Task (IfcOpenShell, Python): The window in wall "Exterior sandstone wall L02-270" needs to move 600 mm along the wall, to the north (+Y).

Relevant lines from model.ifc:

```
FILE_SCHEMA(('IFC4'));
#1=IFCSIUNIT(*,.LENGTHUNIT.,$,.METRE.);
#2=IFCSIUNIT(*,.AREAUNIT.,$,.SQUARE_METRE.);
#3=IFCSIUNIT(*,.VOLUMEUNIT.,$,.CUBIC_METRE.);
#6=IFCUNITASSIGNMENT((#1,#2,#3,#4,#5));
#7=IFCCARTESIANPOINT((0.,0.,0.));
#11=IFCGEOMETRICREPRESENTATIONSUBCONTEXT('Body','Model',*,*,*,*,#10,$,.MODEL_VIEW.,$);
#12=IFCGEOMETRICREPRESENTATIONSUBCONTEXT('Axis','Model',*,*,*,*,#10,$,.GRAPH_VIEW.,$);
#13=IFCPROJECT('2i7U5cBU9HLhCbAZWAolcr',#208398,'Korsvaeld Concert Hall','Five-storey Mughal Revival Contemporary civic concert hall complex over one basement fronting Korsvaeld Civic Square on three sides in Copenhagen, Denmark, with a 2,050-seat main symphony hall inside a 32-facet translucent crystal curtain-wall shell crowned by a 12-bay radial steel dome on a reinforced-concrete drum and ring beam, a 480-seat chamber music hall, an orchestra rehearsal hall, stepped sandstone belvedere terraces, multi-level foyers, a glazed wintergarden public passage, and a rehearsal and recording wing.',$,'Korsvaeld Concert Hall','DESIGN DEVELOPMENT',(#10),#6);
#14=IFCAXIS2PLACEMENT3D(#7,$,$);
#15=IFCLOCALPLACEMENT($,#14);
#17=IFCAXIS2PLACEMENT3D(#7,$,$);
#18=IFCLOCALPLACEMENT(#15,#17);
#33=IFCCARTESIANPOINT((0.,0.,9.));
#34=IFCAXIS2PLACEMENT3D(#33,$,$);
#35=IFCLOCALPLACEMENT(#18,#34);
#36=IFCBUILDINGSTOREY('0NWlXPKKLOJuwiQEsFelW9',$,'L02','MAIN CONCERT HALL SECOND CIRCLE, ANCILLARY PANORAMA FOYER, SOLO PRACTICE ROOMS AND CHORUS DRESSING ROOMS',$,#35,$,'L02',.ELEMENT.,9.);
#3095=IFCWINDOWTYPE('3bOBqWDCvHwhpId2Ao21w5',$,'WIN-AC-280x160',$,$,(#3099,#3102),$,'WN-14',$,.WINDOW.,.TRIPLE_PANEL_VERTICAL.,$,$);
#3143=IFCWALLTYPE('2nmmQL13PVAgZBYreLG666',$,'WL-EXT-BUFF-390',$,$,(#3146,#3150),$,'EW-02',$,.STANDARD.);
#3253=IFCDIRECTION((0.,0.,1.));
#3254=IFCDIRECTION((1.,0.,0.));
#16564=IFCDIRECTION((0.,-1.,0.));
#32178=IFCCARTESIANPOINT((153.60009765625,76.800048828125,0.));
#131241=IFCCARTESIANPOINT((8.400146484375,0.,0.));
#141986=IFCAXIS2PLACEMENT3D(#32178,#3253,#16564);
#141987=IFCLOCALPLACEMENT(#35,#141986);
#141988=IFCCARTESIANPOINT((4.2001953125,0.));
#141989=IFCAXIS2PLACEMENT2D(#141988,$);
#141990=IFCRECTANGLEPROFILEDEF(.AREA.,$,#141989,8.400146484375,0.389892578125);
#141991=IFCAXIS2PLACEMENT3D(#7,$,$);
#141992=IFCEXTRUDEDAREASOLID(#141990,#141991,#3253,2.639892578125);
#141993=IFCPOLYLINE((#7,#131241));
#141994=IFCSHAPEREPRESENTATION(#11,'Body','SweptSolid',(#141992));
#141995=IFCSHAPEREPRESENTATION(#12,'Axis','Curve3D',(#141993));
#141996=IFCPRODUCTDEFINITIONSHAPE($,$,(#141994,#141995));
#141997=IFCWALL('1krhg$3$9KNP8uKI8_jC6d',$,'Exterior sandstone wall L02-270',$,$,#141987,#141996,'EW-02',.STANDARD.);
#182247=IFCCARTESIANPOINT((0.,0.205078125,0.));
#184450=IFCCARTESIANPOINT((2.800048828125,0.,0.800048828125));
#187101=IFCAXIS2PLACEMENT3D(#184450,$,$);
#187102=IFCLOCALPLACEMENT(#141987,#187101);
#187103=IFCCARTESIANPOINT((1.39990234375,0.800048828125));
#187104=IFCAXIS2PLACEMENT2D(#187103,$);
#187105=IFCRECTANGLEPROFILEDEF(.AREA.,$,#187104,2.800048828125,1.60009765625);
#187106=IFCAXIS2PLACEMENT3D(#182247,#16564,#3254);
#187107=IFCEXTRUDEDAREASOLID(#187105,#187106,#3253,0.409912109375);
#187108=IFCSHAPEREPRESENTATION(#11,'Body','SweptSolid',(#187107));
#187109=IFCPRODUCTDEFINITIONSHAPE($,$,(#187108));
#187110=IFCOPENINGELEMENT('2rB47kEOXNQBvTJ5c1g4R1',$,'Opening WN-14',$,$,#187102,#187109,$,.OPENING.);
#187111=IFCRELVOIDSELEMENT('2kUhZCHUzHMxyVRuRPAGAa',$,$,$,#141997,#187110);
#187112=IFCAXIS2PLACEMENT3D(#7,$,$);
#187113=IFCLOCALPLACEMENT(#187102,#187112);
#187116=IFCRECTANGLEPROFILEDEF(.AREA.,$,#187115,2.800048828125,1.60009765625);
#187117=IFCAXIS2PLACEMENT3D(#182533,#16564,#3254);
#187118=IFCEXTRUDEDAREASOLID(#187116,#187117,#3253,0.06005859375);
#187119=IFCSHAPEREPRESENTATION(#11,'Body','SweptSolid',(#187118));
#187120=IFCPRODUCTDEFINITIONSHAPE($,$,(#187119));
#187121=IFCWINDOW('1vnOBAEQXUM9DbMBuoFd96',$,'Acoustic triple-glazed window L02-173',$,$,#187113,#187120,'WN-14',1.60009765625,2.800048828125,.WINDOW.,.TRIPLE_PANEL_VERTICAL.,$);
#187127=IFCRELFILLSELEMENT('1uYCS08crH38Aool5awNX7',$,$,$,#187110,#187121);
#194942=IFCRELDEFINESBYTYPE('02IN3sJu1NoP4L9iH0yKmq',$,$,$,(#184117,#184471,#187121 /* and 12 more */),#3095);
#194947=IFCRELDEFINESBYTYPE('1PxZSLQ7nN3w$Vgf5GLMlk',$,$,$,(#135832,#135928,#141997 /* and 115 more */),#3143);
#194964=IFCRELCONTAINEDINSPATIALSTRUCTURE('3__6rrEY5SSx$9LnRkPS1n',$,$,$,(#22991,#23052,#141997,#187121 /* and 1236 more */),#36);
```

```python
import ifcopenshell
import ifcopenshell.api.geometry
import ifcopenshell.util.placement

model = ifcopenshell.open("model.ifc")

window = model.by_guid("1vnOBAEQXUM9DbMBuoFd96")
opening = window.FillsVoids[0].RelatingOpeningElement
wall = opening.VoidsElements[0].RelatingBuildingElement

wall_matrix = ifcopenshell.util.placement.get_local_placement(wall.ObjectPlacement)
shift = wall_matrix[:3, 0] * -0.6
before = ifcopenshell.util.placement.get_local_placement(window.ObjectPlacement)[:3, 3].copy()

# The window is placed relative to its opening, so it follows when the opening moves.
matrix = ifcopenshell.util.placement.get_local_placement(opening.ObjectPlacement)
matrix[:3, 3] += shift
ifcopenshell.api.geometry.edit_object_placement(
    model, product=opening, matrix=matrix, is_si=False, should_transform_children=True
)

after = ifcopenshell.util.placement.get_local_placement(window.ObjectPlacement)[:3, 3]
print("window moved by", (after - before).round(3) + 0.0)

model.write("model_updated.ifc")
```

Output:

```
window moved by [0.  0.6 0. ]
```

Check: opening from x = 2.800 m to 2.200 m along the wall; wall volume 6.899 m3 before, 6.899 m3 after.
